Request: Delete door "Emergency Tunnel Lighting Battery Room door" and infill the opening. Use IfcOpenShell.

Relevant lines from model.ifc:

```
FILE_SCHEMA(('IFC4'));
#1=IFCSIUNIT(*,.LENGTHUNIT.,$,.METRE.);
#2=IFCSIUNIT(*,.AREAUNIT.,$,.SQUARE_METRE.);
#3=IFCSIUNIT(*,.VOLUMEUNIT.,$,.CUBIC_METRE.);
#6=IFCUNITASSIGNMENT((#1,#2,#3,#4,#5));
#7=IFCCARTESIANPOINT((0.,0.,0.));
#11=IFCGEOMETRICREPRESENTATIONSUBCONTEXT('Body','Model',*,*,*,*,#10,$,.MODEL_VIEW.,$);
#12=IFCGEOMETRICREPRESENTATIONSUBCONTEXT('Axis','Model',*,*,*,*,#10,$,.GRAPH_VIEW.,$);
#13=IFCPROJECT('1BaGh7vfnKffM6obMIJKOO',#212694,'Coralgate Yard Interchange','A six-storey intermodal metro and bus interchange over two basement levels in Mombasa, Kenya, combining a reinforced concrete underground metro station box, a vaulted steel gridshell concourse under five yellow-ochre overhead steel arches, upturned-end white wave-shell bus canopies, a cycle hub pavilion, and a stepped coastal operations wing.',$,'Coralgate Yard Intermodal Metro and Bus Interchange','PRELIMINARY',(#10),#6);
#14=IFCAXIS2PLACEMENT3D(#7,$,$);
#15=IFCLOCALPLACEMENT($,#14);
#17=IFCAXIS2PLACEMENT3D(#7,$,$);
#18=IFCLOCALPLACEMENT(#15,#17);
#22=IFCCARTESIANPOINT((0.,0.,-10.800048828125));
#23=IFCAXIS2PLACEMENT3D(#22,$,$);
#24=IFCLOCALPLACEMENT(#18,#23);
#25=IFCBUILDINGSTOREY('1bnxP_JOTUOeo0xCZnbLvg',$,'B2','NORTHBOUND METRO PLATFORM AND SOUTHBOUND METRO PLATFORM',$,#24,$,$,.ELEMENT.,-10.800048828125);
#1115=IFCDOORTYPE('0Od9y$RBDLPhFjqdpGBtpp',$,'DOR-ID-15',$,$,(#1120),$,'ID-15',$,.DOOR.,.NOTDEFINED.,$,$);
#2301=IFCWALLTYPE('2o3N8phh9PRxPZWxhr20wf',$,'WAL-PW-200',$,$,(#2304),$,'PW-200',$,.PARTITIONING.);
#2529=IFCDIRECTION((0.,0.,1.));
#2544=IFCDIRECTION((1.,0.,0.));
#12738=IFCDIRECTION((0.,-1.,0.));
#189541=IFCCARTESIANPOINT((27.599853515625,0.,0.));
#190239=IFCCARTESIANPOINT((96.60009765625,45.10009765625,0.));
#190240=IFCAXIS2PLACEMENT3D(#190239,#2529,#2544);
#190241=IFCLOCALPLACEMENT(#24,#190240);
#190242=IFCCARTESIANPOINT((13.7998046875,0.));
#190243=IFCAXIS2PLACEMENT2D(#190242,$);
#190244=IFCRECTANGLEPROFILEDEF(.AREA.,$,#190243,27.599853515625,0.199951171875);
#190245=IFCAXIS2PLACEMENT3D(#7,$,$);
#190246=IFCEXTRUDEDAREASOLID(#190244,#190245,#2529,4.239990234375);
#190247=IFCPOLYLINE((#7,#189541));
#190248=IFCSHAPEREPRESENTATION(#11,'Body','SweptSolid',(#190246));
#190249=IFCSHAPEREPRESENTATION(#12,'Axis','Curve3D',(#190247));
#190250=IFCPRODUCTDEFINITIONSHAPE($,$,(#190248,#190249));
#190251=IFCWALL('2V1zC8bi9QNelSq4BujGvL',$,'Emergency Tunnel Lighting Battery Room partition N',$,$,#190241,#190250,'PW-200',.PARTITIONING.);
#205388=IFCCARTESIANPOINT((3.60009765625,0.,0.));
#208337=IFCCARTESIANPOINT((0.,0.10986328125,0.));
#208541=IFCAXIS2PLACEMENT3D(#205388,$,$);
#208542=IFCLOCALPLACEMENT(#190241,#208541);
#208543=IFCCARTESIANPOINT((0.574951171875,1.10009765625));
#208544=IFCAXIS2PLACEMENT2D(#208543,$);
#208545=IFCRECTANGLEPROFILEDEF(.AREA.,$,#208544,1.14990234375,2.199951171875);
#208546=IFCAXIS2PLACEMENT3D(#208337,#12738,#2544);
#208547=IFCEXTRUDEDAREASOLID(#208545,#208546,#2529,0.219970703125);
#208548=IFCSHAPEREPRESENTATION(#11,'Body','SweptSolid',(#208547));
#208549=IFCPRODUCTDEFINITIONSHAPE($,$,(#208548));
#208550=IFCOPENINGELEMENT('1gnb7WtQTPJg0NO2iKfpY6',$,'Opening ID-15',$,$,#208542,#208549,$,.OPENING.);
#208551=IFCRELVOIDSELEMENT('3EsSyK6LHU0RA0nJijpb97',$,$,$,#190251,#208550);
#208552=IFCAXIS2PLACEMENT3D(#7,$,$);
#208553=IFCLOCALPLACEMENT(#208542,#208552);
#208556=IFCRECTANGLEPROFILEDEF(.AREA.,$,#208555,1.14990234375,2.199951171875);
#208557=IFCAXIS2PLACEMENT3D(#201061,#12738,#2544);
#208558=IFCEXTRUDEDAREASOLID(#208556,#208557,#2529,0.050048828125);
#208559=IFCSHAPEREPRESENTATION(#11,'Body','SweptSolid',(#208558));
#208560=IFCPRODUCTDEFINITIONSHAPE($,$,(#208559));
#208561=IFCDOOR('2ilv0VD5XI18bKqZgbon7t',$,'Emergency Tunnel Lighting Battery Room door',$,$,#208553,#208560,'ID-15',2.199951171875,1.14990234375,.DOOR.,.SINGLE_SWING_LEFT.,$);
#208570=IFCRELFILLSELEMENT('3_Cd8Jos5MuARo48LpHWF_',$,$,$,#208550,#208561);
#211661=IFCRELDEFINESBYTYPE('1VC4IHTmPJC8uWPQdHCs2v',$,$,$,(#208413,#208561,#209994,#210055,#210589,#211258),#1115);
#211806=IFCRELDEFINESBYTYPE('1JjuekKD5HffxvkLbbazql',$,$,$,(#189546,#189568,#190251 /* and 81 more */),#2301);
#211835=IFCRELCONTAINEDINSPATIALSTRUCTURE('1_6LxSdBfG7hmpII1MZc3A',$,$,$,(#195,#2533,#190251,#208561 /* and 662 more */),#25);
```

```python
import ifcopenshell
import ifcopenshell.api.feature
import ifcopenshell.api.root
import ifcopenshell.geom
import ifcopenshell.util.shape

model = ifcopenshell.open("model.ifc")
settings = ifcopenshell.geom.settings()


def volume(element):
    """Net volume in cubic metres, openings subtracted."""
    shape = ifcopenshell.geom.create_shape(settings, element)
    return ifcopenshell.util.shape.get_volume(shape.geometry)


door = model.by_guid("2ilv0VD5XI18bKqZgbon7t")
opening = door.FillsVoids[0].RelatingOpeningElement
wall = opening.VoidsElements[0].RelatingBuildingElement
before = volume(wall)

ifcopenshell.api.root.remove_product(model, product=door)
ifcopenshell.api.feature.remove_feature(model, feature=opening)

after = volume(wall)

print(f"wall volume {before:.3f} -> {after:.3f} m3")

model.write("model_rev.ifc")
```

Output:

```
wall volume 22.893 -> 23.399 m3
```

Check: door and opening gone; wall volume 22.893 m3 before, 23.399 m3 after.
